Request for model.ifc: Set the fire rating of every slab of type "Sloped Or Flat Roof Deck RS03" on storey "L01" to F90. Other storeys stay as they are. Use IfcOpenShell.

First a look at what the model holds.

```python
import ifcopenshell
import ifcopenshell.util.element

model = ifcopenshell.open("model.ifc")
print(model.schema)
storey = next(s for s in model.by_type("IfcBuildingStorey") if s.Name == "L01")
slabs = [e for e in ifcopenshell.util.element.get_decomposition(storey) if e.is_a("IfcSlab")]
seen = {}
for e in slabs:
    element_type = ifcopenshell.util.element.get_type(e)
    key = (element_type.Name if element_type != e and element_type else None, ifcopenshell.util.element.get_pset(e, "Pset_SlabCommon", "FireRating"))
    seen[key] = seen.get(key, 0) + 1
for (name, value), count in sorted(seen.items(), key=str):
    print(count, "x", name, "|", value)
```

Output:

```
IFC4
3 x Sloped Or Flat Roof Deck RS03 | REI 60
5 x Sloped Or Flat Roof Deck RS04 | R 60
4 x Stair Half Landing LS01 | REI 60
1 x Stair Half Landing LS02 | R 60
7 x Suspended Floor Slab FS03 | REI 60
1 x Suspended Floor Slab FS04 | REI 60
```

```python
import ifcopenshell
import ifcopenshell.api.pset
import ifcopenshell.util.element

model = ifcopenshell.open("model.ifc")

storey = next(s for s in model.by_type("IfcBuildingStorey") if s.Name == "L01")
slabs = [e for e in ifcopenshell.util.element.get_decomposition(storey) if e.is_a("IfcSlab")]

count = 0
for e in slabs:
    element_type = ifcopenshell.util.element.get_type(e)
    if element_type in (None, e) or element_type.Name != "Sloped Or Flat Roof Deck RS03":
        continue
    # add_pset returns the element's existing set when there is one.
    pset = ifcopenshell.api.pset.add_pset(model, product=e, name="Pset_SlabCommon")
    ifcopenshell.api.pset.edit_pset(model, pset=pset, properties={"FireRating": "F90"})
    count += 1

print(count, "slabs updated")

model.write("model-out.ifc")
```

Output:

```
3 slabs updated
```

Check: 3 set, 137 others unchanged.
